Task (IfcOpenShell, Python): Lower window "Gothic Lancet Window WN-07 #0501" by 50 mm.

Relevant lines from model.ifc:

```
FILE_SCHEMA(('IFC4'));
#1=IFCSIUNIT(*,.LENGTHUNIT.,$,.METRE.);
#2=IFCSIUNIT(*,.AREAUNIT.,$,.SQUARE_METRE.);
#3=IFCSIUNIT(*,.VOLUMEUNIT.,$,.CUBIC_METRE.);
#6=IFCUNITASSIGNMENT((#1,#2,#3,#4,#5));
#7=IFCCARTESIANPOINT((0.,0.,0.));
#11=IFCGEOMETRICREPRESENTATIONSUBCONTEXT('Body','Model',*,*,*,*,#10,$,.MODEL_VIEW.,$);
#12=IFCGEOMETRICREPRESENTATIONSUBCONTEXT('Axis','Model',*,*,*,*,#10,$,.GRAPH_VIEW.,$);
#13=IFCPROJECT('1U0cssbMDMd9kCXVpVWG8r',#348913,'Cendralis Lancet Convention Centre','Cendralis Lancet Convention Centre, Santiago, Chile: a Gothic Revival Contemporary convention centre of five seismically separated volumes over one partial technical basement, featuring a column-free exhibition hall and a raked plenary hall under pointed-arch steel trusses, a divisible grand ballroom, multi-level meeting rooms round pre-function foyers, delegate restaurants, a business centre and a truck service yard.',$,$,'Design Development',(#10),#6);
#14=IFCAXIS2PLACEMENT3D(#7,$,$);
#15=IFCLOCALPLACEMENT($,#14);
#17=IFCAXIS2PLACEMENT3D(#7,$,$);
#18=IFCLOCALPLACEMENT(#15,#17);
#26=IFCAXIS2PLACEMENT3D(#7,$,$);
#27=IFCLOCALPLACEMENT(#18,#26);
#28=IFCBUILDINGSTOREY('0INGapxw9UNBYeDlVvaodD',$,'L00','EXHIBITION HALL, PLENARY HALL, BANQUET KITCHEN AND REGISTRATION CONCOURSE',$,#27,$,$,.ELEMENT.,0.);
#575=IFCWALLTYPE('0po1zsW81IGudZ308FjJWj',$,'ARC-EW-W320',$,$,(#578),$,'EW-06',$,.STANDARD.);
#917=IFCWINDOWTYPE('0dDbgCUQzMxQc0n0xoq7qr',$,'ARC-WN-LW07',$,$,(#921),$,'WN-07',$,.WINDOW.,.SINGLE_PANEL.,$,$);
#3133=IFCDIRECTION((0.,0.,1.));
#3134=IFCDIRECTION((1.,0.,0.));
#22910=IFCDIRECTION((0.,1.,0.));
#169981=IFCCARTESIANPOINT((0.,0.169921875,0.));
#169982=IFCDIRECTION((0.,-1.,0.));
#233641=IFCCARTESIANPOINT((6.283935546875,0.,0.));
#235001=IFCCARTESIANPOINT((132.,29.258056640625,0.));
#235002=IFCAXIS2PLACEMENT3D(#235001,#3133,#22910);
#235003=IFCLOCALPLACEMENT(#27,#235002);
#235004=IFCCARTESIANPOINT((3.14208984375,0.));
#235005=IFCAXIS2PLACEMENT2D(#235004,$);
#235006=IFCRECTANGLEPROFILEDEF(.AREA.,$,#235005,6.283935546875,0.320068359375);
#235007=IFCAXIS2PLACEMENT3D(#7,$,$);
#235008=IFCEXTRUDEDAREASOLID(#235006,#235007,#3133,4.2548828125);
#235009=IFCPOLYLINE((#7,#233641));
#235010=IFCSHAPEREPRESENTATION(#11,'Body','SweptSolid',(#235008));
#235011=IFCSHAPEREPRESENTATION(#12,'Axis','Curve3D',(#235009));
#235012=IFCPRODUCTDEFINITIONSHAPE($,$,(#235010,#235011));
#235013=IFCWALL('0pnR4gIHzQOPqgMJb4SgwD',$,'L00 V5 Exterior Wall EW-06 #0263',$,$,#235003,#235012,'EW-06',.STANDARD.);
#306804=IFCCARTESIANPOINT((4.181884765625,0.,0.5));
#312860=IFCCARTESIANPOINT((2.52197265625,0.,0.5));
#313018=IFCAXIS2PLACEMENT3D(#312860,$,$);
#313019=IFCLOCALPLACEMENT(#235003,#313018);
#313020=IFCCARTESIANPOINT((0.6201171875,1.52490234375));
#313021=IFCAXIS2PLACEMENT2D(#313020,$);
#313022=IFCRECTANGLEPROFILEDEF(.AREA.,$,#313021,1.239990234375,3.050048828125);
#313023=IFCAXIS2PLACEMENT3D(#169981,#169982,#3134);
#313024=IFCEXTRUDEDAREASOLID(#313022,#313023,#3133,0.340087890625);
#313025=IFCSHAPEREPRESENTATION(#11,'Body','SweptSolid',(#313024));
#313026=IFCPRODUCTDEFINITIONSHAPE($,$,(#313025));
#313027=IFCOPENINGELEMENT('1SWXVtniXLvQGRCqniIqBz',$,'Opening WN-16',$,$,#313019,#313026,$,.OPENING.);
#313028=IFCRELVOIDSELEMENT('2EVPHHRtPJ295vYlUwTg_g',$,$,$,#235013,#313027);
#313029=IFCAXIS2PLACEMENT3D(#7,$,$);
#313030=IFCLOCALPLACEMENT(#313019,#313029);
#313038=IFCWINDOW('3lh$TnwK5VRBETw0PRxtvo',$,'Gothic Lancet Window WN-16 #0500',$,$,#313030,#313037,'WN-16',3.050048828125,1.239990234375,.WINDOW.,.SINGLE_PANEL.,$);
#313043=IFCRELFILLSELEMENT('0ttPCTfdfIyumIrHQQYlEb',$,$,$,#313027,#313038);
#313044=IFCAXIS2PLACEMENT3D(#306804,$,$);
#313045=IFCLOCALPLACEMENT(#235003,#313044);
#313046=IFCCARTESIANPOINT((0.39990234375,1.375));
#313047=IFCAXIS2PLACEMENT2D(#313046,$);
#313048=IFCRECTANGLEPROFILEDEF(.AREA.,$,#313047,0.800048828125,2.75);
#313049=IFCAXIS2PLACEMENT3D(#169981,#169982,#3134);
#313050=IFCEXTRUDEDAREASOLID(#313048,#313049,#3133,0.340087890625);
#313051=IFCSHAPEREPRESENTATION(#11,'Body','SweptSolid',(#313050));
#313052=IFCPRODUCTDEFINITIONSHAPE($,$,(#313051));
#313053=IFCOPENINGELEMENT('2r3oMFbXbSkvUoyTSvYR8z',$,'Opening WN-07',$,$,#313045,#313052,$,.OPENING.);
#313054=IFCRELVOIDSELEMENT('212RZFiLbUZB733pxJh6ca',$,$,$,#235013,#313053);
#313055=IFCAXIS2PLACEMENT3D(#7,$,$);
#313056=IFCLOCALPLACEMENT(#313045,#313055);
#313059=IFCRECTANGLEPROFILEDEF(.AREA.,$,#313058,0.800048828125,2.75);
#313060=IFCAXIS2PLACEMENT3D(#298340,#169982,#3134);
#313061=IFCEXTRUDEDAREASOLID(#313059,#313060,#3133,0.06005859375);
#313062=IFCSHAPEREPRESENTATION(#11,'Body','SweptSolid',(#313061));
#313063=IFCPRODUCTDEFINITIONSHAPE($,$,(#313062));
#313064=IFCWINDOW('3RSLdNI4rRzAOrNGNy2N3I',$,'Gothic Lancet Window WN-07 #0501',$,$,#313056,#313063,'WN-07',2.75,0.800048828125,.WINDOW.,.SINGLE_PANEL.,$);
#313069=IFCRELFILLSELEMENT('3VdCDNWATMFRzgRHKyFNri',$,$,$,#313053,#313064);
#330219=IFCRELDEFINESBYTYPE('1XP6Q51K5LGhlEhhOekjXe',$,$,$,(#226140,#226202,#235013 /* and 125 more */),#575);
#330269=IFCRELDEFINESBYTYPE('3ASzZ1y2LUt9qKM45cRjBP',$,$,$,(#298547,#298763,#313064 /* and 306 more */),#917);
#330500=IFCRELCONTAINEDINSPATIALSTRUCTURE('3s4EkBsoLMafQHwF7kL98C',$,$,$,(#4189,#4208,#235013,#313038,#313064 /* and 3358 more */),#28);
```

```python
import numpy as np
import ifcopenshell
import ifcopenshell.api.geometry
import ifcopenshell.util.placement
import ifcopenshell.util.unit

model = ifcopenshell.open("model.ifc")
unit_scale = ifcopenshell.util.unit.calculate_unit_scale(model)

window = model.by_guid("3RSLdNI4rRzAOrNGNy2N3I")
opening = window.FillsVoids[0].RelatingOpeningElement
dz = -0.05

shift = np.array([0.0, 0.0, dz])
# The window is placed relative to its opening, so it follows when the opening moves.
matrix = ifcopenshell.util.placement.get_local_placement(opening.ObjectPlacement)
matrix[:3, 3] += shift
ifcopenshell.api.geometry.edit_object_placement(
    model, product=opening, matrix=matrix, is_si=False, should_transform_children=True
)

print(f"moved by {dz * unit_scale:+.3f} m")

model.write("model_v2.ifc")
```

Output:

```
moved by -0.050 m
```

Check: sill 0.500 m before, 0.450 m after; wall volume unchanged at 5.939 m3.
